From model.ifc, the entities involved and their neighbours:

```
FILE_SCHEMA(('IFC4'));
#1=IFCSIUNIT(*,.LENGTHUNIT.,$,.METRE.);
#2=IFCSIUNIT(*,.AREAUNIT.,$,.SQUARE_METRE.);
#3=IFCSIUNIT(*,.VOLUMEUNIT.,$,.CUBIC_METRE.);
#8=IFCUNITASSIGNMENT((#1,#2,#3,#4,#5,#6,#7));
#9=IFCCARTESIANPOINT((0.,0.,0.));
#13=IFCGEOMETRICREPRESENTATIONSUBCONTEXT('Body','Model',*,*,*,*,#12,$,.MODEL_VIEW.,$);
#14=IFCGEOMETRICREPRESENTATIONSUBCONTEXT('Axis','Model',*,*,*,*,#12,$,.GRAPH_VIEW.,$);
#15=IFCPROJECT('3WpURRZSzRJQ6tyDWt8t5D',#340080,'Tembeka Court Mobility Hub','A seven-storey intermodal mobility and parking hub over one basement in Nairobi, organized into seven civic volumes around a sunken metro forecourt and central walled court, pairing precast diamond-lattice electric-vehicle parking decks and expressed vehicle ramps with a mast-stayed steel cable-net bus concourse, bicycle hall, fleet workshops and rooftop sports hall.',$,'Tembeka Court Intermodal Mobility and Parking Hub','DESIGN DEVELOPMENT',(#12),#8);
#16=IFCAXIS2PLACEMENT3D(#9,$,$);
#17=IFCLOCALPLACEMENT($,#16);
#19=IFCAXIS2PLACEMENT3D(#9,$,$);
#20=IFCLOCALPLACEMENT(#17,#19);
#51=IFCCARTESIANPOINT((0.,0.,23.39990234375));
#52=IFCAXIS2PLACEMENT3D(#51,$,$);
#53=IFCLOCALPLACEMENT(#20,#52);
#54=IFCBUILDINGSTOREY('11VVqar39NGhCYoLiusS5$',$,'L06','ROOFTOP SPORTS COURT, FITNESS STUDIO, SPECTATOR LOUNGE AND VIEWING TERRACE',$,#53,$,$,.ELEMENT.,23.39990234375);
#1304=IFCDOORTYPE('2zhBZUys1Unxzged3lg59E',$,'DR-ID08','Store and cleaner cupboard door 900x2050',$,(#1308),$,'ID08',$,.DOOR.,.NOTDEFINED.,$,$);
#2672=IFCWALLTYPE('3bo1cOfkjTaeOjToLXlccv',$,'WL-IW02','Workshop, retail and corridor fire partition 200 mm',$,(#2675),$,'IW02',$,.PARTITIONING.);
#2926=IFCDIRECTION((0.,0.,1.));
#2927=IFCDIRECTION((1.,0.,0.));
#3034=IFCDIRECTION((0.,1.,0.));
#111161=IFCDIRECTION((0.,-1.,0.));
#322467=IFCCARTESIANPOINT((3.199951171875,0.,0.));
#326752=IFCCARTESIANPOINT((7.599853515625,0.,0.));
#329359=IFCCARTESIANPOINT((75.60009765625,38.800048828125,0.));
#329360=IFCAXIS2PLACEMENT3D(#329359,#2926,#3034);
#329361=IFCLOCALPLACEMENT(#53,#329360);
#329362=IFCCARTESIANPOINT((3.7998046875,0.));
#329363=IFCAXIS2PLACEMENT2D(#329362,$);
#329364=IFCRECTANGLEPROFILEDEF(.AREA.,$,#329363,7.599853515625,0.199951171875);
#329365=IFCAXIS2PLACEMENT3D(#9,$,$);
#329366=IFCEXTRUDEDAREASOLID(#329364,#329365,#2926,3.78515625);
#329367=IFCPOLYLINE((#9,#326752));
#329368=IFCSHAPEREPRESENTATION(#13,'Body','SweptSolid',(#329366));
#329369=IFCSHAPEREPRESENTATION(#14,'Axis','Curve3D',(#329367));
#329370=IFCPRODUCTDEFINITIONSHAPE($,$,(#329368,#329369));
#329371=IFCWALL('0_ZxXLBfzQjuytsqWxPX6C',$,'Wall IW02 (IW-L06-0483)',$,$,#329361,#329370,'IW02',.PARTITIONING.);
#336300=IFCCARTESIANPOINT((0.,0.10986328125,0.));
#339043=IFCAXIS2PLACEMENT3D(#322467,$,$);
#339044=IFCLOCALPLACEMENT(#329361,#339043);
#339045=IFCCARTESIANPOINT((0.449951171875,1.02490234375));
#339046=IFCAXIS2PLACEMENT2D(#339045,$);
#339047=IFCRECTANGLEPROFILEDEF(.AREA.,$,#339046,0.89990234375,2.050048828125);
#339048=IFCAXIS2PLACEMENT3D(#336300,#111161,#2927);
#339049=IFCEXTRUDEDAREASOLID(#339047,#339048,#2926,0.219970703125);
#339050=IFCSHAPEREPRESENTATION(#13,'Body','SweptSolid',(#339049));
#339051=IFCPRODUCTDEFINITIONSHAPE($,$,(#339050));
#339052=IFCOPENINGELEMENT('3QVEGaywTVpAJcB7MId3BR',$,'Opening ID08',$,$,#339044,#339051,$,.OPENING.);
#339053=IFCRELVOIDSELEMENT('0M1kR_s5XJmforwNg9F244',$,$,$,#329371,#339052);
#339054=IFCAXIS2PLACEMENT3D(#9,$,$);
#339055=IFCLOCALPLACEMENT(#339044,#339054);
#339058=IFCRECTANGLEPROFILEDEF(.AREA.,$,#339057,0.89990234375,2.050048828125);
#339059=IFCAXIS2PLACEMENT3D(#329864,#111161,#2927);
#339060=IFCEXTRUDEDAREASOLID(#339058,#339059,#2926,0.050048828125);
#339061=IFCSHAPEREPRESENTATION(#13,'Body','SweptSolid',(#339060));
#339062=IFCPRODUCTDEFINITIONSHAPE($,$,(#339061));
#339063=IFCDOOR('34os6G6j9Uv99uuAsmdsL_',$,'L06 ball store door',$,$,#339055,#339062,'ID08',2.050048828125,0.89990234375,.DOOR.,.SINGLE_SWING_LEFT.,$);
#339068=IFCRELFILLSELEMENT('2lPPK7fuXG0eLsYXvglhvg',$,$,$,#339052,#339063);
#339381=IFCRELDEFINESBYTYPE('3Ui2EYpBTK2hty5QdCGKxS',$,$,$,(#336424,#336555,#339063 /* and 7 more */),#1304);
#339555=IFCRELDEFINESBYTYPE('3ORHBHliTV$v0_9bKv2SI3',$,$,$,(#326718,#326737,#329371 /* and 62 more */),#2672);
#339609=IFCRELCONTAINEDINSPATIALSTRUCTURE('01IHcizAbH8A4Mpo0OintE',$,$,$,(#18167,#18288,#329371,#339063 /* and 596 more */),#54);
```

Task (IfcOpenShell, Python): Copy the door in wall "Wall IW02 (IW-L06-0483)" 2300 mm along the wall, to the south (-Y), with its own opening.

```python
import ifcopenshell
import ifcopenshell.api.feature
import ifcopenshell.api.geometry
import ifcopenshell.api.root
import ifcopenshell.geom
import ifcopenshell.util.element
import ifcopenshell.util.placement
import ifcopenshell.util.shape

model = ifcopenshell.open("model.ifc")
settings = ifcopenshell.geom.settings()


def volume(element):
    """Net volume in cubic metres, openings subtracted."""
    shape = ifcopenshell.geom.create_shape(settings, element)
    return ifcopenshell.util.shape.get_volume(shape.geometry)


door = model.by_guid("34os6G6j9Uv99uuAsmdsL_")
opening = door.FillsVoids[0].RelatingOpeningElement
wall = opening.VoidsElements[0].RelatingBuildingElement
before = volume(wall)
shift = ifcopenshell.util.placement.get_local_placement(wall.ObjectPlacement)[:3, 0] * -2.3

# copy_class copies the void relationship, type, container and properties, but no geometry.
new_opening = ifcopenshell.api.root.copy_class(model, product=opening)
new_opening.Representation = ifcopenshell.util.element.copy_deep(
    model, opening.Representation, exclude=["IfcGeometricRepresentationContext", "IfcRepresentationMap"]
)
new_door = ifcopenshell.api.root.copy_class(model, product=door)
new_door.Representation = ifcopenshell.util.element.copy_deep(
    model, door.Representation, exclude=["IfcGeometricRepresentationContext", "IfcRepresentationMap"]
)
new_door.Tag = None
ifcopenshell.api.feature.add_filling(model, opening=new_opening, element=new_door)

for old, new in ((opening, new_opening), (door, new_door)):
    matrix = ifcopenshell.util.placement.get_local_placement(old.ObjectPlacement)
    matrix[:3, 3] += shift
    ifcopenshell.api.geometry.edit_object_placement(model, product=new, matrix=matrix, is_si=False)

after = volume(wall)

print(f"wall volume {before:.3f} -> {after:.3f} m3")

model.write("model_updated.ifc")
```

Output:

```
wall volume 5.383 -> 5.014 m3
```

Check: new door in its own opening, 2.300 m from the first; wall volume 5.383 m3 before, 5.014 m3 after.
